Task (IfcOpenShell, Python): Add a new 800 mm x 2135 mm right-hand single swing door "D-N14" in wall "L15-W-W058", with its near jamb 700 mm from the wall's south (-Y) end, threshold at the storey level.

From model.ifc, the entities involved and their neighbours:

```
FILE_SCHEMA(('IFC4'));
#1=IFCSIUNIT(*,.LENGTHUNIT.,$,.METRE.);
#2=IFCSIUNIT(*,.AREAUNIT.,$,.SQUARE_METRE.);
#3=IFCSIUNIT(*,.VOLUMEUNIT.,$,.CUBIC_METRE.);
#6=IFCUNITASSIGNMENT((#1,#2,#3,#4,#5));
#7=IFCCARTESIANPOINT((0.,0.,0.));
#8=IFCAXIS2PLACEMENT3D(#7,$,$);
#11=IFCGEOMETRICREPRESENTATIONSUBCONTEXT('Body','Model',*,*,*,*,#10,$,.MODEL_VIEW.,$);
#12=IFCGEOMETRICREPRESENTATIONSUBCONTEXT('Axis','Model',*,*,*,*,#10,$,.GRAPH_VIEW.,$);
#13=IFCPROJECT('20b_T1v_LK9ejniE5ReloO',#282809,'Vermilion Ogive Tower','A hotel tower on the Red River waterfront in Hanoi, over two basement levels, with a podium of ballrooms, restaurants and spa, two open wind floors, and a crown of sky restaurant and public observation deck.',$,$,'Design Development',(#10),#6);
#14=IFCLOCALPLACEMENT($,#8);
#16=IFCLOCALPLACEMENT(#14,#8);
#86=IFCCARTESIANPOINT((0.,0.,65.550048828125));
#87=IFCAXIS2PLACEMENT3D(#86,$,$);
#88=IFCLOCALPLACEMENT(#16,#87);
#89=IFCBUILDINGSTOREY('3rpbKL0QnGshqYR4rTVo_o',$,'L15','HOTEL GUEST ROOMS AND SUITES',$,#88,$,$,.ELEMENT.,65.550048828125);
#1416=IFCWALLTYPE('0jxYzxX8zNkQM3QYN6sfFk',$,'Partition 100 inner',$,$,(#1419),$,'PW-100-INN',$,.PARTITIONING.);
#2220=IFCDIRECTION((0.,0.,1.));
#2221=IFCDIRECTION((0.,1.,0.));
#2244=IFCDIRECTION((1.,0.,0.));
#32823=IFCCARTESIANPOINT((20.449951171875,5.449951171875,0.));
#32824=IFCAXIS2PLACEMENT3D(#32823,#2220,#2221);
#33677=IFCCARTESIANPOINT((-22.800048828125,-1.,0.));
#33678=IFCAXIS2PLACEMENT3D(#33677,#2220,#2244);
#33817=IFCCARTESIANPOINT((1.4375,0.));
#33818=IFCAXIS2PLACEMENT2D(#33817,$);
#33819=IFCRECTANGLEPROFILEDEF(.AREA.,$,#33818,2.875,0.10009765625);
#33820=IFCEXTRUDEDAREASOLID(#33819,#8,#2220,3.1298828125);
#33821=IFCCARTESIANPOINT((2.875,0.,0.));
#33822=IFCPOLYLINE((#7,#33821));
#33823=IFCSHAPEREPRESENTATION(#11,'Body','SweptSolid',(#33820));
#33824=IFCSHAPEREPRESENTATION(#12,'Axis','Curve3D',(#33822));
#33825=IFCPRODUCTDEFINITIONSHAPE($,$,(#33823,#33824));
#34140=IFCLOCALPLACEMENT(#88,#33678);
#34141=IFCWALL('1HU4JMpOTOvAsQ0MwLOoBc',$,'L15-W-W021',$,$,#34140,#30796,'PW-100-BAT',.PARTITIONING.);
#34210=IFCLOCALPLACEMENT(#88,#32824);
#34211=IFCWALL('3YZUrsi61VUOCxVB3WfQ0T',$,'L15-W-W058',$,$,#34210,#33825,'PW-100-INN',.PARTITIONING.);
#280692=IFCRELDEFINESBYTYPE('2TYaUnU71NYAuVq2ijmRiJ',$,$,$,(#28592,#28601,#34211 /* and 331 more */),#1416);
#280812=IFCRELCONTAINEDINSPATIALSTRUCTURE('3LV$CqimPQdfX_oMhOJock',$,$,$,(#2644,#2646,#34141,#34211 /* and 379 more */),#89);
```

```python
import numpy as np
import ifcopenshell
import ifcopenshell.api.feature
import ifcopenshell.api.geometry
import ifcopenshell.api.root
import ifcopenshell.api.spatial
import ifcopenshell.geom
import ifcopenshell.util.element
import ifcopenshell.util.placement
import ifcopenshell.util.representation
import ifcopenshell.util.shape
import ifcopenshell.util.unit

model = ifcopenshell.open("model.ifc")
unit_scale = ifcopenshell.util.unit.calculate_unit_scale(model)
settings = ifcopenshell.geom.settings()


def volume(element):
    """Net volume in cubic metres, openings subtracted."""
    shape = ifcopenshell.geom.create_shape(settings, element)
    return ifcopenshell.util.shape.get_volume(shape.geometry)


wall = model.by_id(34211)
storey = ifcopenshell.util.element.get_container(wall, ifc_class="IfcBuildingStorey")
context = ifcopenshell.util.representation.get_context(model, "Model", "Body", "MODEL_VIEW")
before = volume(wall)

width, height, from_end, sill = 0.8, 2.135, 0.7, 0.0  # metres

# The wall runs along its own X axis, and the end named is its -X end.
wall_shape = ifcopenshell.geom.create_shape(settings, wall)
x, y, z = ifcopenshell.util.shape.get_vertices(wall_shape.geometry).T
start = x.min() + from_end
face, thickness = float(y.min()), float(y.max() - y.min())
wall_matrix = ifcopenshell.util.placement.get_local_placement(wall.ObjectPlacement)
level = ifcopenshell.util.placement.get_local_placement(storey.ObjectPlacement)[2, 3]


def in_wall(x, y):
    """Placement at x, y metres in the wall's axes, at sill height."""
    matrix = wall_matrix.copy()
    matrix[:, 3] = wall_matrix @ np.array([x / unit_scale, y / unit_scale, 0.0, 1.0])
    matrix[2, 3] = level + sill / unit_scale
    return matrix


# Opening: a box that overshoots both wall faces by 50 mm.
opening = ifcopenshell.api.root.create_entity(model, ifc_class="IfcOpeningElement", predefined_type="OPENING")
box = ifcopenshell.api.geometry.add_wall_representation(
    model, context=context, length=width, height=height, thickness=thickness + 0.1
)
ifcopenshell.api.geometry.assign_representation(model, product=opening, representation=box)
ifcopenshell.api.geometry.edit_object_placement(model, product=opening, matrix=in_wall(start, face - 0.05), is_si=False)
ifcopenshell.api.feature.add_feature(model, feature=opening, element=wall)

door = ifcopenshell.api.root.create_entity(model, ifc_class="IfcDoor", name="D-N14", predefined_type="DOOR")
door.OverallWidth, door.OverallHeight = width / unit_scale, height / unit_scale
door.OperationType = "SINGLE_SWING_RIGHT"
body = ifcopenshell.api.geometry.add_door_representation(
    model,
    context=context,
    overall_width=door.OverallWidth,
    overall_height=door.OverallHeight,
    operation_type="SINGLE_SWING_RIGHT",
    lining_properties={"LiningDepth": thickness / unit_scale, "ThresholdDepth": thickness / unit_scale},
)
ifcopenshell.api.geometry.assign_representation(model, product=door, representation=body)
ifcopenshell.api.spatial.assign_container(model, products=[door], relating_structure=storey)
ifcopenshell.api.feature.add_filling(model, opening=opening, element=door)

# The lining spans the wall, so the door starts at the wall face.
ifcopenshell.api.geometry.edit_object_placement(model, product=door, matrix=in_wall(start, face), is_si=False)

after = volume(wall)

print(f"wall volume {before:.3f} -> {after:.3f} m3")

model.write("model_rev.ifc")
```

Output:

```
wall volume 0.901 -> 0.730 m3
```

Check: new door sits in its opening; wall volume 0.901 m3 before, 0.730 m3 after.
